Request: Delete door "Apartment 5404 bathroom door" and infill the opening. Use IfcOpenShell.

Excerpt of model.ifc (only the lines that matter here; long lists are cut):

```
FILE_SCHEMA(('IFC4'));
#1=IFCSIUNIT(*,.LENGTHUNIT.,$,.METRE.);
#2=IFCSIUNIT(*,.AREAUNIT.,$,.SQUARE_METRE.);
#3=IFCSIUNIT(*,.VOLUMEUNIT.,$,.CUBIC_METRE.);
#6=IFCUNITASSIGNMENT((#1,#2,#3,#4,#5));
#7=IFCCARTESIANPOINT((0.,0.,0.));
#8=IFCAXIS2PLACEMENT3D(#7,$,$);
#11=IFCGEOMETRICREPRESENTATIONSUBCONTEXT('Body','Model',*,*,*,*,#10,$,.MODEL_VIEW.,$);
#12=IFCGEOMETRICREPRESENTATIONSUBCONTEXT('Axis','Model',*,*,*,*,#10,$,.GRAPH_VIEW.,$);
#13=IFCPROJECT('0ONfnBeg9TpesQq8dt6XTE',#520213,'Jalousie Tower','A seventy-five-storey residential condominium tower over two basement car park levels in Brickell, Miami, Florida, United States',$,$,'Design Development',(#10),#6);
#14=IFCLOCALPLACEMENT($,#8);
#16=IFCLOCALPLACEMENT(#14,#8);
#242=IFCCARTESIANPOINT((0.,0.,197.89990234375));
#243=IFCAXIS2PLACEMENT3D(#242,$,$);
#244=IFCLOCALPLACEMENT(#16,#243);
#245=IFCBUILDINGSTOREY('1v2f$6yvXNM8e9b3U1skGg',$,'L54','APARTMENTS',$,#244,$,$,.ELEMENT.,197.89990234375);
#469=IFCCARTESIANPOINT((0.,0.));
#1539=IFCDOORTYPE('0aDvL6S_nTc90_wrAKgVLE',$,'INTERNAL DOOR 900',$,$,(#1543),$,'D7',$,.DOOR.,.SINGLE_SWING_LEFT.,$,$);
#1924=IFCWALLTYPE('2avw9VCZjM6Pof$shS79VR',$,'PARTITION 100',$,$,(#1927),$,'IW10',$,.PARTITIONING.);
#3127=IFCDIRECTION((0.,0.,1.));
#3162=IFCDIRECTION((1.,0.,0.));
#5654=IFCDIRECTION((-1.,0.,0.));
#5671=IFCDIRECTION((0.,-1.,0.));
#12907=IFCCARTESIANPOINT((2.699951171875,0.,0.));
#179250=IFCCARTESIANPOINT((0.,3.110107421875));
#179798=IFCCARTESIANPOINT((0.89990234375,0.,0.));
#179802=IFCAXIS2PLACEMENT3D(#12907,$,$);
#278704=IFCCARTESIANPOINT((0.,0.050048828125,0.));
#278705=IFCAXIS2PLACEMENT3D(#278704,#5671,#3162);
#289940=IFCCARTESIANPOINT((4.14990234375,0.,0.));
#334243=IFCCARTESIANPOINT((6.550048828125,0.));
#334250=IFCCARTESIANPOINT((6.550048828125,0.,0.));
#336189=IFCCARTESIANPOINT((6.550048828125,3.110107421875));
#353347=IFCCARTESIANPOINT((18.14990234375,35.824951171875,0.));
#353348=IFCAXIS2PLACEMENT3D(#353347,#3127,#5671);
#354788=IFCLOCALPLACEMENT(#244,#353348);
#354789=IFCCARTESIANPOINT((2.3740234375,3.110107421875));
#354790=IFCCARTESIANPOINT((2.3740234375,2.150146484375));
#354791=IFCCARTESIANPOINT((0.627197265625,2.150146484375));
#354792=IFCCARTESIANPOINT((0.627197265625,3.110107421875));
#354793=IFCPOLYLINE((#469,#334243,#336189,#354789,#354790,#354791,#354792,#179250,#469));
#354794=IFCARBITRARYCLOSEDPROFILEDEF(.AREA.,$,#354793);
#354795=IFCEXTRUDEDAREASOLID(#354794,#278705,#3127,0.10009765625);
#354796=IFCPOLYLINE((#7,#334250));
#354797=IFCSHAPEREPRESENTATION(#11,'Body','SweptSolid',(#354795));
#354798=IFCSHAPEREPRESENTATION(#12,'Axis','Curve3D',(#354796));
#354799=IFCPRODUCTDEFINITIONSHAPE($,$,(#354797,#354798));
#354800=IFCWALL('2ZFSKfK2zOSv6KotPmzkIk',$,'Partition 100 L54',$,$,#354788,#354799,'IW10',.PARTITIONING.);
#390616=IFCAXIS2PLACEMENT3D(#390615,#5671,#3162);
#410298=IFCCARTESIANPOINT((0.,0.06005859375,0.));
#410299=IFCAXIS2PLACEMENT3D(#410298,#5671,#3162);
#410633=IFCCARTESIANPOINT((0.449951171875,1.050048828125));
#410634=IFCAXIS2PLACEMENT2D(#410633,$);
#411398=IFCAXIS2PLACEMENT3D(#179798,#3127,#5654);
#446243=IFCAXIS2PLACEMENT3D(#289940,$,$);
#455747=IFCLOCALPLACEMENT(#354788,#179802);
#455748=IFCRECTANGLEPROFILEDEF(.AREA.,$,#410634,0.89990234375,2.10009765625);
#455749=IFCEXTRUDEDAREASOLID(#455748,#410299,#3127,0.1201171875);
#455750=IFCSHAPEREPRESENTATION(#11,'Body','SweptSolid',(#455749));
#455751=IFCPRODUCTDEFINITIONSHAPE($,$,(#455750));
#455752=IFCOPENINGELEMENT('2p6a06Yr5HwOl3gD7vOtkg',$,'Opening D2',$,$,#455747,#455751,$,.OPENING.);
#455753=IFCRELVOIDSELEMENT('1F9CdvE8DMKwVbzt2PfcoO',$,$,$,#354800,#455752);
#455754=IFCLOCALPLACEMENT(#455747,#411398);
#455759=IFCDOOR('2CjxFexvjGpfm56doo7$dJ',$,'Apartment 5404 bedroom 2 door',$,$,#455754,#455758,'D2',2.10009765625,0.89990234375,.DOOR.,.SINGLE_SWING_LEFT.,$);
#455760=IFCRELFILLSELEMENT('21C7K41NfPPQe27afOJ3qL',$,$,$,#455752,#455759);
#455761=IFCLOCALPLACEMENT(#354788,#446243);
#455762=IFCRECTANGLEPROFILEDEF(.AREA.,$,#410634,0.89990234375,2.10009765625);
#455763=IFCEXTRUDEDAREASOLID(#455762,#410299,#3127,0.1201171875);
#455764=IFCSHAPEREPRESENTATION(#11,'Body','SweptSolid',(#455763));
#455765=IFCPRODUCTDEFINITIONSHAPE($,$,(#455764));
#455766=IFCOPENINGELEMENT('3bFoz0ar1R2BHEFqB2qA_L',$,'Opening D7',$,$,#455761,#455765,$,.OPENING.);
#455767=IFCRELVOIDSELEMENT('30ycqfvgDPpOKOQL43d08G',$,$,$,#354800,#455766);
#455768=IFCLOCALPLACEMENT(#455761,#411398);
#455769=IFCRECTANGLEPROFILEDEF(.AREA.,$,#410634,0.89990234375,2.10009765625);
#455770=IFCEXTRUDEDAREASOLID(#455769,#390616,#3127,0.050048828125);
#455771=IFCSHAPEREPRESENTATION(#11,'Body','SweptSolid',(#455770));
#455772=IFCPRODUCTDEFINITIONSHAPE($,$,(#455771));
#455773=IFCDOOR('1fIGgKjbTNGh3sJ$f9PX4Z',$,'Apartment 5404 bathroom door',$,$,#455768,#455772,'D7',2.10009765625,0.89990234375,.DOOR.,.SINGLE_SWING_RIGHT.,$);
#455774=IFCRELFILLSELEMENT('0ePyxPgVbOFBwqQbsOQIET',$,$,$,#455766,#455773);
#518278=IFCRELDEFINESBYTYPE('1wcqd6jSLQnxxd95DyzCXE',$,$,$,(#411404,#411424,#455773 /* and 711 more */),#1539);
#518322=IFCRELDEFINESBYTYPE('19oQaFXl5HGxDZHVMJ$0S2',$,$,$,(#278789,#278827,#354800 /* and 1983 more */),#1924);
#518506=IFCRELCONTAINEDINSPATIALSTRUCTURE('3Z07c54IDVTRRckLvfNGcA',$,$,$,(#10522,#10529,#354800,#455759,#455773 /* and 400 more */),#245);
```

```python
import ifcopenshell
import ifcopenshell.api.feature
import ifcopenshell.api.root
import ifcopenshell.geom
import ifcopenshell.util.shape

model = ifcopenshell.open("model.ifc")
settings = ifcopenshell.geom.settings()


def volume(element):
    """Net volume in cubic metres, openings subtracted."""
    shape = ifcopenshell.geom.create_shape(settings, element)
    return ifcopenshell.util.shape.get_volume(shape.geometry)


door = model.by_guid("1fIGgKjbTNGh3sJ$f9PX4Z")
opening = door.FillsVoids[0].RelatingOpeningElement
wall = opening.VoidsElements[0].RelatingBuildingElement
before = volume(wall)

ifcopenshell.api.root.remove_product(model, product=door)
ifcopenshell.api.feature.remove_feature(model, feature=opening)

after = volume(wall)

print(f"wall volume {before:.3f} -> {after:.3f} m3")

model.write("model-out.ifc")
```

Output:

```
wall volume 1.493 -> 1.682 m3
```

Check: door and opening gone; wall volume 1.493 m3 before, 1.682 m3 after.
